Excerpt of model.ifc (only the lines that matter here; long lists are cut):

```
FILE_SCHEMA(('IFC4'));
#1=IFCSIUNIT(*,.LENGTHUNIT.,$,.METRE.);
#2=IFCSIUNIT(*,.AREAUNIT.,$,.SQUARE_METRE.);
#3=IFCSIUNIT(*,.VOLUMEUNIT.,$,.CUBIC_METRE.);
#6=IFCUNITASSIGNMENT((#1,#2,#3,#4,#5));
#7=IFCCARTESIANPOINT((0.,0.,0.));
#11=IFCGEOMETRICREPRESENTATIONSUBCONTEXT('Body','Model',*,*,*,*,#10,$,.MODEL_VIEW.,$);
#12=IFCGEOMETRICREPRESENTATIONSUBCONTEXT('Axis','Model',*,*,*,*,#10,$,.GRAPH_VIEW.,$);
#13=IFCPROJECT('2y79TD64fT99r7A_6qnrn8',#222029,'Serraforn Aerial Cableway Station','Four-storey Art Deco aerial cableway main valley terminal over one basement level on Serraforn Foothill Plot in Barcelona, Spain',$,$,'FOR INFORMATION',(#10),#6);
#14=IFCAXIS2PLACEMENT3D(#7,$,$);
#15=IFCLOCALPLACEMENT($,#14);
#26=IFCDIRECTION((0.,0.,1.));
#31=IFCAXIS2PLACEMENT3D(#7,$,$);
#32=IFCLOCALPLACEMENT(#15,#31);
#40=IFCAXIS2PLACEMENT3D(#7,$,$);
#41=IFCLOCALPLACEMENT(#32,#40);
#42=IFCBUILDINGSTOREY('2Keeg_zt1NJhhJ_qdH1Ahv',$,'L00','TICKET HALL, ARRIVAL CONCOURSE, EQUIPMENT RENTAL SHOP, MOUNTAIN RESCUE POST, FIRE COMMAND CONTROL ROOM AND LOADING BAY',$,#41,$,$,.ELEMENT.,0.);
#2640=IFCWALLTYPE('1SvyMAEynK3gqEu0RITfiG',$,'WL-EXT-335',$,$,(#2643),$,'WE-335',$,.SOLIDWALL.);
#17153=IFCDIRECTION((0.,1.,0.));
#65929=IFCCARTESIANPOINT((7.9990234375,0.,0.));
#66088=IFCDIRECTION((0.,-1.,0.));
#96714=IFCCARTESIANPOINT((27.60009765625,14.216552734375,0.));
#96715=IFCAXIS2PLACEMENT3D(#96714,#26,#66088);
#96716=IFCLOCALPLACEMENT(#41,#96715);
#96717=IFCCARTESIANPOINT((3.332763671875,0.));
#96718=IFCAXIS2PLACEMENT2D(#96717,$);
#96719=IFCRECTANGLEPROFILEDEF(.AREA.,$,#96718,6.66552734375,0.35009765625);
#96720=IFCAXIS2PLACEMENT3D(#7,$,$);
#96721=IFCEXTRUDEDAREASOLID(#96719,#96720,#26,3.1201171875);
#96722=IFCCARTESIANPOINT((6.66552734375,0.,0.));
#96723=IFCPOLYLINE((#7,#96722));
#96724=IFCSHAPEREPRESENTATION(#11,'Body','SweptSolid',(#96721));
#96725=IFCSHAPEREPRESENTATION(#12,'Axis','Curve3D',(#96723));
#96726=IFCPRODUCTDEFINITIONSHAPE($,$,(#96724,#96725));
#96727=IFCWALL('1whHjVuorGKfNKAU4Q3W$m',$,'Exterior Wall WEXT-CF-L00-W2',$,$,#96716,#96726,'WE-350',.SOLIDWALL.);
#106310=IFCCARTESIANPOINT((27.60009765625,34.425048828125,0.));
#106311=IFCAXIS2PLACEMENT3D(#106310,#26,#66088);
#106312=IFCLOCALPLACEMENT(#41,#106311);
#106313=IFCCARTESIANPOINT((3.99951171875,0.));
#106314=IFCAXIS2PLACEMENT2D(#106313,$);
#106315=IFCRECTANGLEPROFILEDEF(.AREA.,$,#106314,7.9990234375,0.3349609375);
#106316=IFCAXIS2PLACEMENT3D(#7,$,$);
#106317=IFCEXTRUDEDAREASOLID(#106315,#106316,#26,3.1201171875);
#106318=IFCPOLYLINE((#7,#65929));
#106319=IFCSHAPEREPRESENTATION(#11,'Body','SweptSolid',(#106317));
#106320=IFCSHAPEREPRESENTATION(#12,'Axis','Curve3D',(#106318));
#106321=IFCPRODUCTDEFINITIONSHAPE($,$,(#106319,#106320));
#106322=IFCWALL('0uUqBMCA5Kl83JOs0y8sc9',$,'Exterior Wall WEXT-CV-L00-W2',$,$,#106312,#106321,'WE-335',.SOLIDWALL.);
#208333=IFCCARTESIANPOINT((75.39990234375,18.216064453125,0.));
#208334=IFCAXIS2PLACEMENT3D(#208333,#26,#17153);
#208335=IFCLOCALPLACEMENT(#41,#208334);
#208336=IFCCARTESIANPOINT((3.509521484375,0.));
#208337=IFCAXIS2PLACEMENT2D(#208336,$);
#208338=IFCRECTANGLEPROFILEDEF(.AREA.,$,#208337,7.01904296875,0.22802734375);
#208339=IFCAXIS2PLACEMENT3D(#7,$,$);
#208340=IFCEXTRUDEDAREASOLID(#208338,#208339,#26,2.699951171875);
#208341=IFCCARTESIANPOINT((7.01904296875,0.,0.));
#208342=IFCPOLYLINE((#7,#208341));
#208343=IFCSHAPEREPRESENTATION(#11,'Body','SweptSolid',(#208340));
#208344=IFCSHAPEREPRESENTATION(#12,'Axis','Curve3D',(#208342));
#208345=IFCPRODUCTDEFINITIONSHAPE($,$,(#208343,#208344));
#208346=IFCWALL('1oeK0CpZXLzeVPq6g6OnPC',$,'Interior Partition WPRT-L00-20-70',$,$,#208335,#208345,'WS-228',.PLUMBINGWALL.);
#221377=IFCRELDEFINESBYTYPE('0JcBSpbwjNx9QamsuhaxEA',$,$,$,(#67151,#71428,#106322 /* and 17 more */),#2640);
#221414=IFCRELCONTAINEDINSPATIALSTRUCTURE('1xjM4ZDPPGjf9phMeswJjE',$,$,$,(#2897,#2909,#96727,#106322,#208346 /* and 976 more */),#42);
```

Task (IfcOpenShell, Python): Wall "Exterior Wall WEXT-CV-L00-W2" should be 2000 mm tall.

```python
import ifcopenshell
import ifcopenshell.geom
import ifcopenshell.util.representation
import ifcopenshell.util.shape

model = ifcopenshell.open("model.ifc")
settings = ifcopenshell.geom.settings()


def volume(element):
    """Net volume in cubic metres, openings subtracted."""
    shape = ifcopenshell.geom.create_shape(settings, element)
    return ifcopenshell.util.shape.get_volume(shape.geometry)


wall = model.by_guid("0uUqBMCA5Kl83JOs0y8sc9")
before = volume(wall)

body = ifcopenshell.util.representation.get_representation(wall, "Model", "Body")
solid = body.Items[0]
old_height = solid.Depth
solid.Depth = 2.0
after = volume(wall)

print(f"height {old_height:g} -> {solid.Depth:g}, volume {before:.3f} -> {after:.3f} m3")

model.write("model_v2.ifc")
```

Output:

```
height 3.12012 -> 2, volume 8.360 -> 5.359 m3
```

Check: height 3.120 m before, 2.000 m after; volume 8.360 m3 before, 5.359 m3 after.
